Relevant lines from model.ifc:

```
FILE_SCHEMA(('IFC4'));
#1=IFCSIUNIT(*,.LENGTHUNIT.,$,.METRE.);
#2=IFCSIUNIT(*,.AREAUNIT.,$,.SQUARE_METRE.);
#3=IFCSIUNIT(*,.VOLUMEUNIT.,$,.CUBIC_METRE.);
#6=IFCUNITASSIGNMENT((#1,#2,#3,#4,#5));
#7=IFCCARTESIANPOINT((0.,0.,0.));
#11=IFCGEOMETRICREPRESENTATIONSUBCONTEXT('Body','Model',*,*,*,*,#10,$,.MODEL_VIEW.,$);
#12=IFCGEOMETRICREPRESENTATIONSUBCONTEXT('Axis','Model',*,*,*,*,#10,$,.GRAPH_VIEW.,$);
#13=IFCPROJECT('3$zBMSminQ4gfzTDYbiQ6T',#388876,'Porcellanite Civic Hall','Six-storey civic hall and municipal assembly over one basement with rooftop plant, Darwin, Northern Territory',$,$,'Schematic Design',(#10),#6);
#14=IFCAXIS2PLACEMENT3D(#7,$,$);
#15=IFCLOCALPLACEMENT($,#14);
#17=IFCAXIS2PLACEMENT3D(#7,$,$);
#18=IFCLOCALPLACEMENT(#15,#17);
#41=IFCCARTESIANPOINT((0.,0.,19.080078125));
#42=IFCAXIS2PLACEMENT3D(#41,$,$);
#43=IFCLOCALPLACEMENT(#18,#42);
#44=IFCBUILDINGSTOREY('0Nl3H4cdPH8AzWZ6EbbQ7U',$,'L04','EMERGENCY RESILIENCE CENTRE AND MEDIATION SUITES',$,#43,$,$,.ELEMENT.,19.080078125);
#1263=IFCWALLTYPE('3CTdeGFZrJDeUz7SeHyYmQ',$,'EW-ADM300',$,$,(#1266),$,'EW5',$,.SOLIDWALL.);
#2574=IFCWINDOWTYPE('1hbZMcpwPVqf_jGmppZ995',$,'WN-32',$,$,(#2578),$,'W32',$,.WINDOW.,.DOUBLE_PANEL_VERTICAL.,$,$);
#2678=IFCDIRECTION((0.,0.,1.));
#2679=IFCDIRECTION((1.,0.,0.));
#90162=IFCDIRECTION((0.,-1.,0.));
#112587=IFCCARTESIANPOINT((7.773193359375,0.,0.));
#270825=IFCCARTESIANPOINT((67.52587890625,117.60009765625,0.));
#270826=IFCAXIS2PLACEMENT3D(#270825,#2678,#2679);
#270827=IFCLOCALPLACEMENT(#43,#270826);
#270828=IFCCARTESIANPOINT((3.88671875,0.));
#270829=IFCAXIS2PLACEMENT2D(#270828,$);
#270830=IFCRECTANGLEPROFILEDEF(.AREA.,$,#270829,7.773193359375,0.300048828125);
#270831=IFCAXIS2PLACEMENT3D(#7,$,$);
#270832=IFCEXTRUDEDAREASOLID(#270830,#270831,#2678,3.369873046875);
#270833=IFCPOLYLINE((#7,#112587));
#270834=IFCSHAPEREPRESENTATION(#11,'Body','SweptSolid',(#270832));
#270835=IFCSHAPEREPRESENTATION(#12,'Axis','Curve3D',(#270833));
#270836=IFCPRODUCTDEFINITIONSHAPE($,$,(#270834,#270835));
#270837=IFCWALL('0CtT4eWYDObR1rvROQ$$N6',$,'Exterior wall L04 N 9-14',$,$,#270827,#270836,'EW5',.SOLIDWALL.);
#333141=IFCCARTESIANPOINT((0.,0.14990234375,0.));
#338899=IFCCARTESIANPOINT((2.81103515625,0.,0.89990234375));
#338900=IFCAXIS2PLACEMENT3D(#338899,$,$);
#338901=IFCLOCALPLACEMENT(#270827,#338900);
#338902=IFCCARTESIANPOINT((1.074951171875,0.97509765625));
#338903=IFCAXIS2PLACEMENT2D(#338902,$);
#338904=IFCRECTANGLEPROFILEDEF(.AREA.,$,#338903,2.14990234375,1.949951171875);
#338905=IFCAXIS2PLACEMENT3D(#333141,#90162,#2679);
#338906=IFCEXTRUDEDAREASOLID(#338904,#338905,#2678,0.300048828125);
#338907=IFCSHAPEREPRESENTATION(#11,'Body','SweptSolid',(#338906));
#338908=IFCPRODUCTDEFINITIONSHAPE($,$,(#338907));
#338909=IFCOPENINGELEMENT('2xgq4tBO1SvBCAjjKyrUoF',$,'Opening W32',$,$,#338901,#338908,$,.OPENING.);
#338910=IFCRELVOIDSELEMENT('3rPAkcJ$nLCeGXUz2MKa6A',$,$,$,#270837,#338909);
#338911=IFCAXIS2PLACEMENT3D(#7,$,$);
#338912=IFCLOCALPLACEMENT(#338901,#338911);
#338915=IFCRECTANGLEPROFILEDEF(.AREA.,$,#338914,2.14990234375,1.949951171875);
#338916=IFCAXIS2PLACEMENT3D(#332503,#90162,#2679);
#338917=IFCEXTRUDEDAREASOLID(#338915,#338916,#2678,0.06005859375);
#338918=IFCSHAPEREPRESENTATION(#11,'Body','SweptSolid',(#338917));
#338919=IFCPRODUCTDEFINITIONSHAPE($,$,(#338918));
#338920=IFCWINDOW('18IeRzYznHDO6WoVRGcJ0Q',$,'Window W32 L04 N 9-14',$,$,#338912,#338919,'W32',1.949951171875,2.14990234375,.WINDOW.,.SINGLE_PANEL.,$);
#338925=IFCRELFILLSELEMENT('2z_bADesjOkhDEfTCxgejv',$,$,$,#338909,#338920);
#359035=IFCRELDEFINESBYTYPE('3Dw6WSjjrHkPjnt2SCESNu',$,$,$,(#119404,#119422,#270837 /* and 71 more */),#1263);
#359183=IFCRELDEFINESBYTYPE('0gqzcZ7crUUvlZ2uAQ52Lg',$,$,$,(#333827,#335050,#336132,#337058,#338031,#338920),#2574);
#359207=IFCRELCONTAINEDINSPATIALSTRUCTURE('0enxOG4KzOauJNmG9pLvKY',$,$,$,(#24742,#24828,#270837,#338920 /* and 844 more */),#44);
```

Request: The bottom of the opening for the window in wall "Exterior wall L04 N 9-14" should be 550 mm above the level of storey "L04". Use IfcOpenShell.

```python
import numpy as np
import ifcopenshell
import ifcopenshell.api.geometry
import ifcopenshell.geom
import ifcopenshell.util.element
import ifcopenshell.util.placement
import ifcopenshell.util.shape
import ifcopenshell.util.unit

model = ifcopenshell.open("model.ifc")
unit_scale = ifcopenshell.util.unit.calculate_unit_scale(model)

window = model.by_guid("18IeRzYznHDO6WoVRGcJ0Q")
opening = window.FillsVoids[0].RelatingOpeningElement
storey = ifcopenshell.util.element.get_container(window, ifc_class="IfcBuildingStorey")
level = ifcopenshell.util.placement.get_local_placement(storey.ObjectPlacement)[2, 3]

# The opening's origin need not be at the sill, so measure its lowest point.
shape = ifcopenshell.geom.create_shape(ifcopenshell.geom.settings(), opening)
bottom = ifcopenshell.util.shape.get_shape_bottom_elevation(shape, shape.geometry) / unit_scale
dz = level + 0.55 / unit_scale - bottom

shift = np.array([0.0, 0.0, dz])
# The window is placed relative to its opening, so it follows when the opening moves.
matrix = ifcopenshell.util.placement.get_local_placement(opening.ObjectPlacement)
matrix[:3, 3] += shift
ifcopenshell.api.geometry.edit_object_placement(
    model, product=opening, matrix=matrix, is_si=False, should_transform_children=True
)

print(f"moved by {dz * unit_scale:+.3f} m")

model.write("model_updated.ifc")
```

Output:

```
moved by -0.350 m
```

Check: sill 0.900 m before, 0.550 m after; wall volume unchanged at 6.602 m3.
